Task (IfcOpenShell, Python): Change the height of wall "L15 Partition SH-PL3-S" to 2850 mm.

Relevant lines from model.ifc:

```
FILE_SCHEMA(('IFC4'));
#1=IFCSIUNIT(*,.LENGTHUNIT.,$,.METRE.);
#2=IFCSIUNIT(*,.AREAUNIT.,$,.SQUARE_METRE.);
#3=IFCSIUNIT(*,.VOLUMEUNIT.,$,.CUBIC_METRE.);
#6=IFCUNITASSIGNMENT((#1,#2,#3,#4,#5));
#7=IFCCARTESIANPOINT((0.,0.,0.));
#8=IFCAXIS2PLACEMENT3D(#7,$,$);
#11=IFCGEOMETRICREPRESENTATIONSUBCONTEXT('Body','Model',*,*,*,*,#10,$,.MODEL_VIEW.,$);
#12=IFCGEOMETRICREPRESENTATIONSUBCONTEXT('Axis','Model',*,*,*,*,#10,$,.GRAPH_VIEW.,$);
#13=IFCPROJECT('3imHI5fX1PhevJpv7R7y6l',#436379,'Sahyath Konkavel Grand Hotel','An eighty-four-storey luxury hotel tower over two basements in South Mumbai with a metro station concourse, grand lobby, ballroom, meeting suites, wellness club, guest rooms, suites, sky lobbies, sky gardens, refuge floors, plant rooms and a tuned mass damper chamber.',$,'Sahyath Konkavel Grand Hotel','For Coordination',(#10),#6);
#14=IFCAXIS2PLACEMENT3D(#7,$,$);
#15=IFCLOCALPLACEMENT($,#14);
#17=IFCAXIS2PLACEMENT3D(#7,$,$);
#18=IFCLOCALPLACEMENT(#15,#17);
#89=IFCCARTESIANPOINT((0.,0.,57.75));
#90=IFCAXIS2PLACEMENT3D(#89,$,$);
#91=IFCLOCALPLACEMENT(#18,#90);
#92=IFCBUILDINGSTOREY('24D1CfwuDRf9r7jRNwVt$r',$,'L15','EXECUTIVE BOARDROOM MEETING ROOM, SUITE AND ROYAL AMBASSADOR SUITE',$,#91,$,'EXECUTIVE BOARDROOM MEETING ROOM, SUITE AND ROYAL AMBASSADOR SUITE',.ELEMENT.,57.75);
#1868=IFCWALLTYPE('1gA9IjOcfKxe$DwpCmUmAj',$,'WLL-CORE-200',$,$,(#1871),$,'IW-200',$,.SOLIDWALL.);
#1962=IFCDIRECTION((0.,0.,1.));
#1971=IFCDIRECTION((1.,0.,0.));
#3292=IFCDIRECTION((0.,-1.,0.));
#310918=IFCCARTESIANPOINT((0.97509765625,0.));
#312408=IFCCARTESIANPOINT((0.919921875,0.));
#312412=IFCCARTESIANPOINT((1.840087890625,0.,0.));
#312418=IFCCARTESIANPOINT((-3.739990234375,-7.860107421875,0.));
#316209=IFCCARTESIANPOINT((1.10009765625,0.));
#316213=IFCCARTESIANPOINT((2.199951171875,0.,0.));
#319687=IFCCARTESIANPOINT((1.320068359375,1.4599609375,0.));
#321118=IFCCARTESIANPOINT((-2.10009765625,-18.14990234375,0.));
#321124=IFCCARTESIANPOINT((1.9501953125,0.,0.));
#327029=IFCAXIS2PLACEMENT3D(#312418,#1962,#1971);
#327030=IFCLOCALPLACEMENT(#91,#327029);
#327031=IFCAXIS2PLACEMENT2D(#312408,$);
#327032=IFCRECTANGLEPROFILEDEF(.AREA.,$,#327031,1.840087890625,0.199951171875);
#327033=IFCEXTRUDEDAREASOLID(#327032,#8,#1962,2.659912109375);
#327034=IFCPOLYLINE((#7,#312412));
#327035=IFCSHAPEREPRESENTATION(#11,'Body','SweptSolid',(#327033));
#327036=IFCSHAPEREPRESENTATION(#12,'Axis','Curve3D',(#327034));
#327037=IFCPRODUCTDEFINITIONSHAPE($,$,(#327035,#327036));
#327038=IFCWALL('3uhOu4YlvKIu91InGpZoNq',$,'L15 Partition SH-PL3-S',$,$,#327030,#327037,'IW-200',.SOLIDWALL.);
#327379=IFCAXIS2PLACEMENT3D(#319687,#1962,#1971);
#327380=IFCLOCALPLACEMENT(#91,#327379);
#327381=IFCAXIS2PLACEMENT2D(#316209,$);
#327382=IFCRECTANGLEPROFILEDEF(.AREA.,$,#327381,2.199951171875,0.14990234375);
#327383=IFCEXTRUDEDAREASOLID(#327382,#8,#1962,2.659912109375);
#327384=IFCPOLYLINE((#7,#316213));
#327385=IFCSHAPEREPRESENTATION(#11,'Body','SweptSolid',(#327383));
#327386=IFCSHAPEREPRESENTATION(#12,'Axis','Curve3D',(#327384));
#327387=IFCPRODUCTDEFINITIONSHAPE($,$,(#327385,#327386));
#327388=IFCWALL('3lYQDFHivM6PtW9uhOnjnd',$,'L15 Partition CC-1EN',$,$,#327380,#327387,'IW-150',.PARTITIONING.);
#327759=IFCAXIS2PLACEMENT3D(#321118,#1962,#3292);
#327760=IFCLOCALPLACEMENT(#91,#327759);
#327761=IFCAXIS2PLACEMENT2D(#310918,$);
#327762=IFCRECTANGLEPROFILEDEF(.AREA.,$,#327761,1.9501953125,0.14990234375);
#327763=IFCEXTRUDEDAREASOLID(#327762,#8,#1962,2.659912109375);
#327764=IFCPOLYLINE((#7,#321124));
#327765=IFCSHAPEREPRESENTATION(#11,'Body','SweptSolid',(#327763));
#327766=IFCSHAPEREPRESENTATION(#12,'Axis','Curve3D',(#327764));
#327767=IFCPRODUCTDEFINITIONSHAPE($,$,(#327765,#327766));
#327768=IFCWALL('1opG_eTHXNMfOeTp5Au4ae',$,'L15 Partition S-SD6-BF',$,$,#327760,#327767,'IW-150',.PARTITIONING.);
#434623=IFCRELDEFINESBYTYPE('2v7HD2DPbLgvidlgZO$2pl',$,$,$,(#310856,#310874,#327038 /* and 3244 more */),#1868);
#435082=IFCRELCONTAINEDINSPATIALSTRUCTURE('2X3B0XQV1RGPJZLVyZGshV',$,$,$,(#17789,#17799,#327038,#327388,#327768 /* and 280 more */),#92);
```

```python
import ifcopenshell
import ifcopenshell.geom
import ifcopenshell.util.representation
import ifcopenshell.util.shape
import ifcopenshell.util.unit

model = ifcopenshell.open("model.ifc")
unit_scale = ifcopenshell.util.unit.calculate_unit_scale(model)
settings = ifcopenshell.geom.settings()


def volume(element):
    """Net volume in cubic metres, openings subtracted."""
    shape = ifcopenshell.geom.create_shape(settings, element)
    return ifcopenshell.util.shape.get_volume(shape.geometry)


wall = model.by_guid("3uhOu4YlvKIu91InGpZoNq")
before = volume(wall)

body = ifcopenshell.util.representation.get_representation(wall, "Model", "Body")
solid = body.Items[0]
old_height = solid.Depth
solid.Depth = 2.85 / unit_scale
after = volume(wall)

print(f"height {old_height:g} -> {solid.Depth:g}, volume {before:.3f} -> {after:.3f} m3")

model.write("model_edited.ifc")
```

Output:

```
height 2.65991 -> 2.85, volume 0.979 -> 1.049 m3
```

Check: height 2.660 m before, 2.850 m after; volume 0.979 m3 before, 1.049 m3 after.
